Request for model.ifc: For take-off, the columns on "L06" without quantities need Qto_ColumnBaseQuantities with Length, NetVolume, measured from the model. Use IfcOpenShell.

First a look at what the model holds.

```python
import ifcopenshell
import ifcopenshell.util.element
import ifcopenshell.util.unit

model = ifcopenshell.open("model.ifc")
print(model.schema)
for unit_type in ("LENGTHUNIT", "AREAUNIT", "VOLUMEUNIT"):
    print(unit_type, ifcopenshell.util.unit.calculate_unit_scale(model, unit_type))
storey = next(s for s in model.by_type("IfcBuildingStorey") if s.Name == "L06")
columns = [e for e in ifcopenshell.util.element.get_decomposition(storey) if e.is_a("IfcColumn")]
for e in sorted(columns, key=lambda e: e.id()):
    print(e.id(), e.is_a(), e.Name, list(ifcopenshell.util.element.get_psets(e, qtos_only=True)), sep=" | ")
```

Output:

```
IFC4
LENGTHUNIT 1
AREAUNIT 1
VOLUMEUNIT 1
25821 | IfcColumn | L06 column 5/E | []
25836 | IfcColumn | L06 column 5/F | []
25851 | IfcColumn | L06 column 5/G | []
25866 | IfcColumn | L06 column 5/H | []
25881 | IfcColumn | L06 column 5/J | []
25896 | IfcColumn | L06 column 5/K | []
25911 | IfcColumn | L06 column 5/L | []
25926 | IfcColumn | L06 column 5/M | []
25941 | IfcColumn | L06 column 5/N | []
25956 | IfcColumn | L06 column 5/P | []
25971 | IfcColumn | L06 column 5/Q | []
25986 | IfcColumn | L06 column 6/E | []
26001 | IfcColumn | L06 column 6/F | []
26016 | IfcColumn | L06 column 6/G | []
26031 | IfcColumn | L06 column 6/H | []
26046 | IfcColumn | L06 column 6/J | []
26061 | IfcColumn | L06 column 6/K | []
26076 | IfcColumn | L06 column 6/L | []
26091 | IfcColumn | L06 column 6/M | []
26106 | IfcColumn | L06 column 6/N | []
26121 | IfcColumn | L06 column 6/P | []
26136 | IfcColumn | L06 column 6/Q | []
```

```python
import ifcopenshell
import ifcopenshell.api.pset
import ifcopenshell.geom
import ifcopenshell.util.element
import ifcopenshell.util.shape
import ifcopenshell.util.unit

model = ifcopenshell.open("model.ifc")
unit_scale = ifcopenshell.util.unit.calculate_unit_scale(model)
volume_scale = ifcopenshell.util.unit.calculate_unit_scale(model, "VOLUMEUNIT")
settings = ifcopenshell.geom.settings()

storey = next(s for s in model.by_type("IfcBuildingStorey") if s.Name == "L06")
columns = [e for e in ifcopenshell.util.element.get_decomposition(storey) if e.is_a("IfcColumn")]

for e in sorted(columns, key=lambda e: e.id()):
    if ifcopenshell.util.element.get_psets(e, qtos_only=True, should_inherit=False):
        continue
    # Geometry comes back in metres, in the element's own axes.
    shape = ifcopenshell.geom.create_shape(settings, e)
    values = {
        "Length": ifcopenshell.util.shape.get_z(shape.geometry) / unit_scale,
        "NetVolume": ifcopenshell.util.shape.get_volume(shape.geometry) / volume_scale,
    }
    qto = ifcopenshell.api.pset.add_qto(model, product=e, name="Qto_ColumnBaseQuantities")
    ifcopenshell.api.pset.edit_qto(model, qto=qto, properties=values)
    print(e.id(), {k: round(v, 3) for k, v in values.items()})

model.write("model_v2.ifc")
```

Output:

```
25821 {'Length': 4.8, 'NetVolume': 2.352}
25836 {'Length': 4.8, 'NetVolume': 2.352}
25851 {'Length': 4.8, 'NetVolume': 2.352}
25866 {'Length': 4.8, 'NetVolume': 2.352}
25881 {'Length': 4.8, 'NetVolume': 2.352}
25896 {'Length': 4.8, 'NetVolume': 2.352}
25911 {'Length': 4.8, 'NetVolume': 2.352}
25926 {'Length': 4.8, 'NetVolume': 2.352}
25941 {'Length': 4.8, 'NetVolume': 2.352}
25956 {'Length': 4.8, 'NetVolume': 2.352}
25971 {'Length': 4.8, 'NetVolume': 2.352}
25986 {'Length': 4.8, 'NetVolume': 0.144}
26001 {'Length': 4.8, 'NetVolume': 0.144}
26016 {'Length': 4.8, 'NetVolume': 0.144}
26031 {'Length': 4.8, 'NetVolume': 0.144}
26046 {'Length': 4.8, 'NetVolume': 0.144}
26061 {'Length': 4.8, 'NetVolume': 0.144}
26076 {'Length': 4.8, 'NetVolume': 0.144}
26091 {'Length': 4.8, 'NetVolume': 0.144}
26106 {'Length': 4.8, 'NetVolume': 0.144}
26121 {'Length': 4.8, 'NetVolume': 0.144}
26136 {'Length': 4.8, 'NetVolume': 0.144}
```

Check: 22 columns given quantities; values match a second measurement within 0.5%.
